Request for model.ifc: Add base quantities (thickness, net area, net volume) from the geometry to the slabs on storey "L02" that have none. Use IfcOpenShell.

First a look at what the model holds.

```python
import ifcopenshell
import ifcopenshell.util.element
import ifcopenshell.util.unit

model = ifcopenshell.open("model.ifc")
print(model.schema)
for unit_type in ("LENGTHUNIT", "AREAUNIT", "VOLUMEUNIT"):
    print(unit_type, ifcopenshell.util.unit.calculate_unit_scale(model, unit_type))
storey = next(s for s in model.by_type("IfcBuildingStorey") if s.Name == "L02")
slabs = [e for e in ifcopenshell.util.element.get_decomposition(storey) if e.is_a("IfcSlab")]
for e in sorted(slabs, key=lambda e: e.id()):
    print(e.id(), e.is_a(), e.Name, list(ifcopenshell.util.element.get_psets(e, qtos_only=True)), sep=" | ")
```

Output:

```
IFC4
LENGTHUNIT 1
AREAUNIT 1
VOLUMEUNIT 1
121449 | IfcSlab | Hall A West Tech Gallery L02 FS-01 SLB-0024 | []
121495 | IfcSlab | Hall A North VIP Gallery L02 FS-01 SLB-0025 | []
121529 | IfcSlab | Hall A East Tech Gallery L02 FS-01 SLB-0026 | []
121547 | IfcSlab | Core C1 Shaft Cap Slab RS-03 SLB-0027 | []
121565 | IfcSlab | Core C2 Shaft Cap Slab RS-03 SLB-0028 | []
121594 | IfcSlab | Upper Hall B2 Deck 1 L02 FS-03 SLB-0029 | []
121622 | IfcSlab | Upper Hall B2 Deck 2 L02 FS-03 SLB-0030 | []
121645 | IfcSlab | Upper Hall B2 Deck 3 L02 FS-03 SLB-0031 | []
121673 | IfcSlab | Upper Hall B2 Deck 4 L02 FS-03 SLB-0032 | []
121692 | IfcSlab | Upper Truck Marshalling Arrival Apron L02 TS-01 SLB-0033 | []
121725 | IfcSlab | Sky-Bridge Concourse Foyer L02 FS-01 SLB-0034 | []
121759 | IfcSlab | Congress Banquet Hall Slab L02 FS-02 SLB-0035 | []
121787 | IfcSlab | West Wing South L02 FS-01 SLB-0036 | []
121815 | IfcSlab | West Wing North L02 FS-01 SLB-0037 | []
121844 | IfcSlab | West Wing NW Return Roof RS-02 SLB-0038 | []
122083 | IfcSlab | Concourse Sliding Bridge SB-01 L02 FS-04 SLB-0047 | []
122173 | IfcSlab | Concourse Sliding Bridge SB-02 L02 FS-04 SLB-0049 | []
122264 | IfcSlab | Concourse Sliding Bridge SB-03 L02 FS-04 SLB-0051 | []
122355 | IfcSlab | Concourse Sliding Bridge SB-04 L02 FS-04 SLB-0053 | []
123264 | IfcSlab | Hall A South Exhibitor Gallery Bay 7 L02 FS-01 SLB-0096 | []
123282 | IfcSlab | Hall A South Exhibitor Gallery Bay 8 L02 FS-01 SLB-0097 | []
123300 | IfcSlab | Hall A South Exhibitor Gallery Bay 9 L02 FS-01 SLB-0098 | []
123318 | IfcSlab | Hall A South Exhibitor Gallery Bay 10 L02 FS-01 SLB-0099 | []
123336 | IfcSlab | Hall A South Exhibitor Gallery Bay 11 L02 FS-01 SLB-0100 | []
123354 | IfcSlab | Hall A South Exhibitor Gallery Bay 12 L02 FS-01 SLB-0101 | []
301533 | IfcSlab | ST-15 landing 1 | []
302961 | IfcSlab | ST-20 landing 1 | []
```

```python
import ifcopenshell
import ifcopenshell.api.pset
import ifcopenshell.geom
import ifcopenshell.util.element
import ifcopenshell.util.shape
import ifcopenshell.util.unit

model = ifcopenshell.open("model.ifc")
unit_scale = ifcopenshell.util.unit.calculate_unit_scale(model)
area_scale = ifcopenshell.util.unit.calculate_unit_scale(model, "AREAUNIT")
volume_scale = ifcopenshell.util.unit.calculate_unit_scale(model, "VOLUMEUNIT")
settings = ifcopenshell.geom.settings()

storey = next(s for s in model.by_type("IfcBuildingStorey") if s.Name == "L02")
slabs = [e for e in ifcopenshell.util.element.get_decomposition(storey) if e.is_a("IfcSlab")]

for e in sorted(slabs, key=lambda e: e.id()):
    if ifcopenshell.util.element.get_psets(e, qtos_only=True, should_inherit=False):
        continue
    # Geometry comes back in metres, in the element's own axes.
    shape = ifcopenshell.geom.create_shape(settings, e)
    values = {
        "Width": ifcopenshell.util.shape.get_z(shape.geometry) / unit_scale,
        "NetArea": ifcopenshell.util.shape.get_footprint_area(shape.geometry) / area_scale,
        "NetVolume": ifcopenshell.util.shape.get_volume(shape.geometry) / volume_scale,
    }
    qto = ifcopenshell.api.pset.add_qto(model, product=e, name="Qto_SlabBaseQuantities")
    ifcopenshell.api.pset.edit_qto(model, qto=qto, properties=values)
    print(e.id(), {k: round(v, 3) for k, v in values.items()})

model.write("model-out.ifc")
```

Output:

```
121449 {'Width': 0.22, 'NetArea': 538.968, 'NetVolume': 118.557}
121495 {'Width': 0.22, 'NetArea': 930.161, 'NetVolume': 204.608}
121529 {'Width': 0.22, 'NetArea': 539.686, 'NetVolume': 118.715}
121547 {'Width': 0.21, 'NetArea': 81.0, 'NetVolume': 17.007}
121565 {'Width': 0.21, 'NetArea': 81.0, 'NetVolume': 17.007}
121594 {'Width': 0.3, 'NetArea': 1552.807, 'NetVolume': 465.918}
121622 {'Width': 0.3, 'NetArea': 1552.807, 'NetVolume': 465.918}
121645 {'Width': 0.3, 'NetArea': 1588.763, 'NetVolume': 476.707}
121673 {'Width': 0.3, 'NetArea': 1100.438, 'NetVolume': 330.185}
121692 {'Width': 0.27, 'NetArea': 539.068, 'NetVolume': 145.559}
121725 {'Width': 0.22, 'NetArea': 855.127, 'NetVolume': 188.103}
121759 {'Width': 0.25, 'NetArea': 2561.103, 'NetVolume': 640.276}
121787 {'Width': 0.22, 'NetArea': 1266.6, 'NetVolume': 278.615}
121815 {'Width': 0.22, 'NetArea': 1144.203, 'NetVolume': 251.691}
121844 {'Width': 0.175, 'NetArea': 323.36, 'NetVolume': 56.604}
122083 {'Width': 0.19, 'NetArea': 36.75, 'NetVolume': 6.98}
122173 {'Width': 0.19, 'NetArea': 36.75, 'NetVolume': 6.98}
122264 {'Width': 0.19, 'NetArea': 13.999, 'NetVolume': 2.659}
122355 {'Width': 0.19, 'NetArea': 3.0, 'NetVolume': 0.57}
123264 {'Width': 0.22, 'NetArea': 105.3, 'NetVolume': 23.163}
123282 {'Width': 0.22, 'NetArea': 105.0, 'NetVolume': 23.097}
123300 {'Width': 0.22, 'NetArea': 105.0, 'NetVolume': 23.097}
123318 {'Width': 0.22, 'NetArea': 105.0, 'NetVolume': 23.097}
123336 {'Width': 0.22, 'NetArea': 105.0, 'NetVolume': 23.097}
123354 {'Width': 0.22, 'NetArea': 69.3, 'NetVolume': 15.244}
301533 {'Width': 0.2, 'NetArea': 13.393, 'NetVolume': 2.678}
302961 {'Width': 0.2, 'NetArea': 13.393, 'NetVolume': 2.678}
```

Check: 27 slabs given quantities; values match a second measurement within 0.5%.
